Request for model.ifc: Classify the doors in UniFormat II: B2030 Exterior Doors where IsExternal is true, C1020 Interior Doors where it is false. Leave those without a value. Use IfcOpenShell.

First a look at what the model holds.

```python
import ifcopenshell
import ifcopenshell.util.element

model = ifcopenshell.open("model.ifc")
print(model.schema)
print("classifications:", [c.Name for c in model.by_type("IfcClassification")])
values = [ifcopenshell.util.element.get_pset(e, "Pset_DoorCommon", "IsExternal") for e in model.by_type("IfcDoor")]
for value in (True, False, None):
    print("IsExternal", value, values.count(value))
```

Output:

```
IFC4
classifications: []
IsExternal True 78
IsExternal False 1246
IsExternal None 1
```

```python
import ifcopenshell
import ifcopenshell.api.classification
import ifcopenshell.util.element

model = ifcopenshell.open("model.ifc")

system = ifcopenshell.api.classification.add_classification(model, classification="UniFormat II")

doors = model.by_type("IfcDoor")
external = {e: ifcopenshell.util.element.get_pset(e, "Pset_DoorCommon", "IsExternal") for e in doors}
for flag, code, name in ((True, "B2030", "Exterior Doors"), (False, "C1020", "Interior Doors")):
    products = [e for e in doors if external[e] is flag]
    ifcopenshell.api.classification.add_reference(
        model, products=products, classification=system, identification=code, name=name
    )
    print(code, len(products))

model.write("model_v2.ifc")
```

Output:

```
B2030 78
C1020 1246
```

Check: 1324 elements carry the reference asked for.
